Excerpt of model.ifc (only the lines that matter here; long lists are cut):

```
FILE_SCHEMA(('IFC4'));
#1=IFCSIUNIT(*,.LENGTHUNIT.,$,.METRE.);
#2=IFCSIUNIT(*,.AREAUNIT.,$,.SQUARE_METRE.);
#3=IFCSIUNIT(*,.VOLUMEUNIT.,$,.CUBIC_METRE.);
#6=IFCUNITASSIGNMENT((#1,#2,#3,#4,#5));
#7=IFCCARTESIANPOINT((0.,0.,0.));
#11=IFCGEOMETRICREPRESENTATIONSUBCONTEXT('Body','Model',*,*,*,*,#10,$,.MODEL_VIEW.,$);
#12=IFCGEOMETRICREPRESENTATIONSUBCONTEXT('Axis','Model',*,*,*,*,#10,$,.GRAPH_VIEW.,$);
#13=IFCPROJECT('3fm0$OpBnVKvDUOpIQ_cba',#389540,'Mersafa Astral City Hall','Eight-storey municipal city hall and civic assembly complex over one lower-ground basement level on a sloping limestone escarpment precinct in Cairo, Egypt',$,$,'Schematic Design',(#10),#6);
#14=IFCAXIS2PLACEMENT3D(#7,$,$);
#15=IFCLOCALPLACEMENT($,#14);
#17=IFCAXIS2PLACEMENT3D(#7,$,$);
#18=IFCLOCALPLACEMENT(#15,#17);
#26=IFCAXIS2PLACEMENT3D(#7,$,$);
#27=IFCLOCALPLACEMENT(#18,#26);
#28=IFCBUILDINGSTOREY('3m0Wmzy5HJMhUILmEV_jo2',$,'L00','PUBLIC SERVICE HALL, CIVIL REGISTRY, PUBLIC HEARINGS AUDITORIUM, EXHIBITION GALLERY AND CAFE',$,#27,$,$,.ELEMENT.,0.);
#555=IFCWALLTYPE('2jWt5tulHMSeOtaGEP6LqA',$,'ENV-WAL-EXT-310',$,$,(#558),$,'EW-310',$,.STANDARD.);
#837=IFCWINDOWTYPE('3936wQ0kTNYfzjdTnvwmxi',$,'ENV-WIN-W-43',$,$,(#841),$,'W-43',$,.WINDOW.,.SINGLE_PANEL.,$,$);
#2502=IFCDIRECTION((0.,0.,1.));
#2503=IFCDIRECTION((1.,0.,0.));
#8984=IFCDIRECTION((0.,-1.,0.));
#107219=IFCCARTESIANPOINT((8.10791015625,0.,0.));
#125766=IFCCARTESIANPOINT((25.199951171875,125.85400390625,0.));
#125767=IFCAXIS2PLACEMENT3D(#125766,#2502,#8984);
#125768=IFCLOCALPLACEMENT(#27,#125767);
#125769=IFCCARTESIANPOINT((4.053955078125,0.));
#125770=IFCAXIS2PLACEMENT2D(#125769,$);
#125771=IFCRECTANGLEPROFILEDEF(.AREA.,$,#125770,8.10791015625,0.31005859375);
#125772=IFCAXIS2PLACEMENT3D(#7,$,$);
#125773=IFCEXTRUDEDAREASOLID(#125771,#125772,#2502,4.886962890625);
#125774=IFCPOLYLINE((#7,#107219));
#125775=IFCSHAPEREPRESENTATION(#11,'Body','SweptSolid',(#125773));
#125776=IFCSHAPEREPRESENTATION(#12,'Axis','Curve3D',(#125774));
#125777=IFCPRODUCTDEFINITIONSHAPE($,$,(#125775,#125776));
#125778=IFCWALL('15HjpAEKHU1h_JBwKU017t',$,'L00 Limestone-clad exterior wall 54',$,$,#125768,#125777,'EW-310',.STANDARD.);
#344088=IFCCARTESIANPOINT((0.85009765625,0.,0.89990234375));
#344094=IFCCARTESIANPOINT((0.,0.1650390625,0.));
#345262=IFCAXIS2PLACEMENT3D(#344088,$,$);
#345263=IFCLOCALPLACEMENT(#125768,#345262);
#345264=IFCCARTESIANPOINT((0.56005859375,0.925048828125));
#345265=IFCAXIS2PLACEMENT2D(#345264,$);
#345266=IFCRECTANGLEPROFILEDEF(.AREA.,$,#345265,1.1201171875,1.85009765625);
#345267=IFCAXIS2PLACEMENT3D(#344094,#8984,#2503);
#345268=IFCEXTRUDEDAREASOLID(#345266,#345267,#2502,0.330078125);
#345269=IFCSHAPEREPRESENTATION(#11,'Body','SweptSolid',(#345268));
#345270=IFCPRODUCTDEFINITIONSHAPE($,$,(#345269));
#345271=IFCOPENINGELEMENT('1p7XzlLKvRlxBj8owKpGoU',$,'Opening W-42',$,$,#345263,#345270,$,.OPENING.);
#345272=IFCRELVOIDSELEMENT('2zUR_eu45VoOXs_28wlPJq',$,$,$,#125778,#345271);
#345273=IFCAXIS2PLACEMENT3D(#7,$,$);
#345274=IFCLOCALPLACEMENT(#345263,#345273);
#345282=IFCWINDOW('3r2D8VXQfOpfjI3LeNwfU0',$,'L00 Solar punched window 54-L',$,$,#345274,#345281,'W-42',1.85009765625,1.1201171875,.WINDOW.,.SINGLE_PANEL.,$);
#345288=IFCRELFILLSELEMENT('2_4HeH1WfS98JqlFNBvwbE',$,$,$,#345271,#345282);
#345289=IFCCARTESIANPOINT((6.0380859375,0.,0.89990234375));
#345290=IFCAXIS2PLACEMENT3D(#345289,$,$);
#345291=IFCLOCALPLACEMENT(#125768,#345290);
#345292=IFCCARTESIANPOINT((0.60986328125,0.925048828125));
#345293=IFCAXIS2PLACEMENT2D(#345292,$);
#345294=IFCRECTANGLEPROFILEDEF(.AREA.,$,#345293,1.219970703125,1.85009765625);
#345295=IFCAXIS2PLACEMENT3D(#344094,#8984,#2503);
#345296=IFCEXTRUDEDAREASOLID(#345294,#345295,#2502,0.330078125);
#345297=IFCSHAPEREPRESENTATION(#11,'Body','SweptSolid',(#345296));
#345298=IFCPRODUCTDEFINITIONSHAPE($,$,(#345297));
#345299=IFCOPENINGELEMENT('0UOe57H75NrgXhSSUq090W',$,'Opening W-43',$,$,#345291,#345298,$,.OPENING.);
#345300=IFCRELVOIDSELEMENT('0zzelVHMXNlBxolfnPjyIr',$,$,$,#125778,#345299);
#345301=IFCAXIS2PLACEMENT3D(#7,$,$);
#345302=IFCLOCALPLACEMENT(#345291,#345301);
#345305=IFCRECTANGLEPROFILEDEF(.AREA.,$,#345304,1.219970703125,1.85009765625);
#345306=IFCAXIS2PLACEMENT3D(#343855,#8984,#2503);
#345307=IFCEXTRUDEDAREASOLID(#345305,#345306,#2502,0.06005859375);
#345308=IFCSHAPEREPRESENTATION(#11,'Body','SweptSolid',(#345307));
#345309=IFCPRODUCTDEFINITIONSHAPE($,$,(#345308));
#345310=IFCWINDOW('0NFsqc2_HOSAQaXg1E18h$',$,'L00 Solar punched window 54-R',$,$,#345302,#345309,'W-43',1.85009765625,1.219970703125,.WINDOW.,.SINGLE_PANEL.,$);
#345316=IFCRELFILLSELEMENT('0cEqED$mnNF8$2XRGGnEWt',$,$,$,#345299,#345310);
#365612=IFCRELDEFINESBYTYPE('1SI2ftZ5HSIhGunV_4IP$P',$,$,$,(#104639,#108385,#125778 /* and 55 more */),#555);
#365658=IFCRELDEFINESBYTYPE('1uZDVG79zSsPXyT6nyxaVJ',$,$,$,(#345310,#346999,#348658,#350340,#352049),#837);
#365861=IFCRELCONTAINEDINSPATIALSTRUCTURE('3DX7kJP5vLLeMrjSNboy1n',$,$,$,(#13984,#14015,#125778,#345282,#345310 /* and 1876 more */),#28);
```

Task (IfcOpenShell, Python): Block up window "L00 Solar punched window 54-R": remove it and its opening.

```python
import ifcopenshell
import ifcopenshell.api.feature
import ifcopenshell.api.root
import ifcopenshell.geom
import ifcopenshell.util.shape

model = ifcopenshell.open("model.ifc")
settings = ifcopenshell.geom.settings()


def volume(element):
    """Net volume in cubic metres, openings subtracted."""
    shape = ifcopenshell.geom.create_shape(settings, element)
    return ifcopenshell.util.shape.get_volume(shape.geometry)


window = model.by_guid("0NFsqc2_HOSAQaXg1E18h$")
opening = window.FillsVoids[0].RelatingOpeningElement
wall = opening.VoidsElements[0].RelatingBuildingElement
before = volume(wall)

ifcopenshell.api.root.remove_product(model, product=window)
ifcopenshell.api.feature.remove_feature(model, feature=opening)

after = volume(wall)

print(f"wall volume {before:.3f} -> {after:.3f} m3")

model.write("model_edited.ifc")
```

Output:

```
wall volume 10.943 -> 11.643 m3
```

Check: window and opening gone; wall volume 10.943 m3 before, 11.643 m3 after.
